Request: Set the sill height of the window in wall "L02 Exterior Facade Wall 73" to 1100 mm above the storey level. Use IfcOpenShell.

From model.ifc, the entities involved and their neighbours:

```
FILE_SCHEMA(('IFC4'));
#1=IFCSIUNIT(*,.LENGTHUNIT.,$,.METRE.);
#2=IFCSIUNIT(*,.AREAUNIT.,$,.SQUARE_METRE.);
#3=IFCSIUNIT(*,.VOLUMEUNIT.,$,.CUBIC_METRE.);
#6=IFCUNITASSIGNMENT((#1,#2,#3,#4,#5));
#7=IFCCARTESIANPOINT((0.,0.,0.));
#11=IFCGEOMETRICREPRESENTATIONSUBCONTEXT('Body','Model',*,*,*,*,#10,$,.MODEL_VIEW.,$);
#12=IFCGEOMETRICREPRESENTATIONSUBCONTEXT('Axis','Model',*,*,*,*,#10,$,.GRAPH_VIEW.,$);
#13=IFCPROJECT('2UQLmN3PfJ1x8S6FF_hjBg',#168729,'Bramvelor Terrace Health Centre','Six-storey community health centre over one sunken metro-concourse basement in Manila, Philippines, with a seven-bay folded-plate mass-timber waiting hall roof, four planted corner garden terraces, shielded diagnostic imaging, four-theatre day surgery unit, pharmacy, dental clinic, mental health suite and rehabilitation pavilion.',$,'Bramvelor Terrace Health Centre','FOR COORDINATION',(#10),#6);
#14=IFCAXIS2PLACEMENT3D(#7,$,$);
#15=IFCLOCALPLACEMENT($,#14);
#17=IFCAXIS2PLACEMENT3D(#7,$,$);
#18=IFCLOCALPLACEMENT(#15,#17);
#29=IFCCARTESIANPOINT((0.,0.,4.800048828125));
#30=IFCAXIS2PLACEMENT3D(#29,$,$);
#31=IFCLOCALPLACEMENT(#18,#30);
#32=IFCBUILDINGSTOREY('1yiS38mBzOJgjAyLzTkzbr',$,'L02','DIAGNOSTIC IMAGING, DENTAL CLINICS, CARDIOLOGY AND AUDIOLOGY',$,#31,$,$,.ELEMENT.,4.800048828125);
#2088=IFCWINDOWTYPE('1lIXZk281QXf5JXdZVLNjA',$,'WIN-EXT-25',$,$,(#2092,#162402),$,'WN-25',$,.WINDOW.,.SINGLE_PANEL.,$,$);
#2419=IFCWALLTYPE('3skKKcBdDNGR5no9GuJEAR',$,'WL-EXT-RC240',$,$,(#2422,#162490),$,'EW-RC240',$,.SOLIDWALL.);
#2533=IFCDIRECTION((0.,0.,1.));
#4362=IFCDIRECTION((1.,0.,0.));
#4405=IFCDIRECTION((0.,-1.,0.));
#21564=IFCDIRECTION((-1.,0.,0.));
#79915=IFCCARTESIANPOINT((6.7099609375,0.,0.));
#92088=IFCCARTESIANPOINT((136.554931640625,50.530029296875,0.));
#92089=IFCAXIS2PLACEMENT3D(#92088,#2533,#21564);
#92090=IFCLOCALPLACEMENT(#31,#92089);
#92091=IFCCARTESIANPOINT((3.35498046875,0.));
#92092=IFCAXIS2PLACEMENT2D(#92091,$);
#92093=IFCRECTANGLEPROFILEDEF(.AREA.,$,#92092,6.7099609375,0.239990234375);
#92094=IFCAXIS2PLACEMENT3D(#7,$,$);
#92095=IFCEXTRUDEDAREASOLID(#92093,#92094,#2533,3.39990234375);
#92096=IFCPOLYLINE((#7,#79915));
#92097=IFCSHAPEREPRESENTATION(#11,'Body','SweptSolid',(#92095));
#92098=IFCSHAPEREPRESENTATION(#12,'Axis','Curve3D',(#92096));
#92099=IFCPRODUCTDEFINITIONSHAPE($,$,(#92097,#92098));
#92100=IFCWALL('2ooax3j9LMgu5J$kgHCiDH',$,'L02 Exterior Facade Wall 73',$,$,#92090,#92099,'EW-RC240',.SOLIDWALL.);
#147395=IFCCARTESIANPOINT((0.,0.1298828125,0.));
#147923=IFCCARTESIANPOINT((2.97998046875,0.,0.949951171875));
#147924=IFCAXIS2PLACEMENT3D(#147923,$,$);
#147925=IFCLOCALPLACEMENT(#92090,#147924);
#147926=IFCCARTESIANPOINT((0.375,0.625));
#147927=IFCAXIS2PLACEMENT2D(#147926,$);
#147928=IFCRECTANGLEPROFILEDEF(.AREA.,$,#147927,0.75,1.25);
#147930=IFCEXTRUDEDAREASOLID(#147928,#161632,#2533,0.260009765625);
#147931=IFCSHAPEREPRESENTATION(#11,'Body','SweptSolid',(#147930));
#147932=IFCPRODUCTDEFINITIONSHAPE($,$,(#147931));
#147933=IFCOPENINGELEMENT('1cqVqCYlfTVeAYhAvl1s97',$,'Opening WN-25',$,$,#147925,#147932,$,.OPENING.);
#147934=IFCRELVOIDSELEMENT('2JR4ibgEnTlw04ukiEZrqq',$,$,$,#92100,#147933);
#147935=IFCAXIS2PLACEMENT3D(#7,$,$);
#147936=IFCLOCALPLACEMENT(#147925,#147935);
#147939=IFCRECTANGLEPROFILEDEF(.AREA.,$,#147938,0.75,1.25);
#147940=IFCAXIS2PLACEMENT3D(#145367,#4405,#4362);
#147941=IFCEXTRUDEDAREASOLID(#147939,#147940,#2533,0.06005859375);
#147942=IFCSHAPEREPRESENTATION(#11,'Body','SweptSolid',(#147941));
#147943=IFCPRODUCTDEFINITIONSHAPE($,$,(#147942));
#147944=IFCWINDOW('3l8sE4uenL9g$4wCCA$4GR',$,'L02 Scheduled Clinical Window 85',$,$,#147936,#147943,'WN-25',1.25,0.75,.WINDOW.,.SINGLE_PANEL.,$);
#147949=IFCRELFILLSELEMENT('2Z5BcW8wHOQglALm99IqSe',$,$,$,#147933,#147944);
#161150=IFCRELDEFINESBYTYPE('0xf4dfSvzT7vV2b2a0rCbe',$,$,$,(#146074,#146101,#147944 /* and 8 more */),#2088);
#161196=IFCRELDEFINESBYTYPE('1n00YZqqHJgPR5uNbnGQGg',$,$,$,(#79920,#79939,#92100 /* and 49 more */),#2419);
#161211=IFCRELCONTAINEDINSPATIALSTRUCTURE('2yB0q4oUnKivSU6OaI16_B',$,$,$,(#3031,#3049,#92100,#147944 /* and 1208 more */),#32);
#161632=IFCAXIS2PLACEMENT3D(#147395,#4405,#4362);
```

```python
import numpy as np
import ifcopenshell
import ifcopenshell.api.geometry
import ifcopenshell.geom
import ifcopenshell.util.element
import ifcopenshell.util.placement
import ifcopenshell.util.shape
import ifcopenshell.util.unit

model = ifcopenshell.open("model.ifc")
unit_scale = ifcopenshell.util.unit.calculate_unit_scale(model)

window = model.by_guid("3l8sE4uenL9g$4wCCA$4GR")
opening = window.FillsVoids[0].RelatingOpeningElement
storey = ifcopenshell.util.element.get_container(window, ifc_class="IfcBuildingStorey")
level = ifcopenshell.util.placement.get_local_placement(storey.ObjectPlacement)[2, 3]

# The opening's origin need not be at the sill, so measure its lowest point.
shape = ifcopenshell.geom.create_shape(ifcopenshell.geom.settings(), opening)
bottom = ifcopenshell.util.shape.get_shape_bottom_elevation(shape, shape.geometry) / unit_scale
dz = level + 1.1 - bottom

shift = np.array([0.0, 0.0, dz])
# The window is placed relative to its opening, so it follows when the opening moves.
matrix = ifcopenshell.util.placement.get_local_placement(opening.ObjectPlacement)
matrix[:3, 3] += shift
ifcopenshell.api.geometry.edit_object_placement(
    model, product=opening, matrix=matrix, is_si=False, should_transform_children=True
)

print(f"moved by {dz * unit_scale:+.3f} m")

model.write("model_rev.ifc")
```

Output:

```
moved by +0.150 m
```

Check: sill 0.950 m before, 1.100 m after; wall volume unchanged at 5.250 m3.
